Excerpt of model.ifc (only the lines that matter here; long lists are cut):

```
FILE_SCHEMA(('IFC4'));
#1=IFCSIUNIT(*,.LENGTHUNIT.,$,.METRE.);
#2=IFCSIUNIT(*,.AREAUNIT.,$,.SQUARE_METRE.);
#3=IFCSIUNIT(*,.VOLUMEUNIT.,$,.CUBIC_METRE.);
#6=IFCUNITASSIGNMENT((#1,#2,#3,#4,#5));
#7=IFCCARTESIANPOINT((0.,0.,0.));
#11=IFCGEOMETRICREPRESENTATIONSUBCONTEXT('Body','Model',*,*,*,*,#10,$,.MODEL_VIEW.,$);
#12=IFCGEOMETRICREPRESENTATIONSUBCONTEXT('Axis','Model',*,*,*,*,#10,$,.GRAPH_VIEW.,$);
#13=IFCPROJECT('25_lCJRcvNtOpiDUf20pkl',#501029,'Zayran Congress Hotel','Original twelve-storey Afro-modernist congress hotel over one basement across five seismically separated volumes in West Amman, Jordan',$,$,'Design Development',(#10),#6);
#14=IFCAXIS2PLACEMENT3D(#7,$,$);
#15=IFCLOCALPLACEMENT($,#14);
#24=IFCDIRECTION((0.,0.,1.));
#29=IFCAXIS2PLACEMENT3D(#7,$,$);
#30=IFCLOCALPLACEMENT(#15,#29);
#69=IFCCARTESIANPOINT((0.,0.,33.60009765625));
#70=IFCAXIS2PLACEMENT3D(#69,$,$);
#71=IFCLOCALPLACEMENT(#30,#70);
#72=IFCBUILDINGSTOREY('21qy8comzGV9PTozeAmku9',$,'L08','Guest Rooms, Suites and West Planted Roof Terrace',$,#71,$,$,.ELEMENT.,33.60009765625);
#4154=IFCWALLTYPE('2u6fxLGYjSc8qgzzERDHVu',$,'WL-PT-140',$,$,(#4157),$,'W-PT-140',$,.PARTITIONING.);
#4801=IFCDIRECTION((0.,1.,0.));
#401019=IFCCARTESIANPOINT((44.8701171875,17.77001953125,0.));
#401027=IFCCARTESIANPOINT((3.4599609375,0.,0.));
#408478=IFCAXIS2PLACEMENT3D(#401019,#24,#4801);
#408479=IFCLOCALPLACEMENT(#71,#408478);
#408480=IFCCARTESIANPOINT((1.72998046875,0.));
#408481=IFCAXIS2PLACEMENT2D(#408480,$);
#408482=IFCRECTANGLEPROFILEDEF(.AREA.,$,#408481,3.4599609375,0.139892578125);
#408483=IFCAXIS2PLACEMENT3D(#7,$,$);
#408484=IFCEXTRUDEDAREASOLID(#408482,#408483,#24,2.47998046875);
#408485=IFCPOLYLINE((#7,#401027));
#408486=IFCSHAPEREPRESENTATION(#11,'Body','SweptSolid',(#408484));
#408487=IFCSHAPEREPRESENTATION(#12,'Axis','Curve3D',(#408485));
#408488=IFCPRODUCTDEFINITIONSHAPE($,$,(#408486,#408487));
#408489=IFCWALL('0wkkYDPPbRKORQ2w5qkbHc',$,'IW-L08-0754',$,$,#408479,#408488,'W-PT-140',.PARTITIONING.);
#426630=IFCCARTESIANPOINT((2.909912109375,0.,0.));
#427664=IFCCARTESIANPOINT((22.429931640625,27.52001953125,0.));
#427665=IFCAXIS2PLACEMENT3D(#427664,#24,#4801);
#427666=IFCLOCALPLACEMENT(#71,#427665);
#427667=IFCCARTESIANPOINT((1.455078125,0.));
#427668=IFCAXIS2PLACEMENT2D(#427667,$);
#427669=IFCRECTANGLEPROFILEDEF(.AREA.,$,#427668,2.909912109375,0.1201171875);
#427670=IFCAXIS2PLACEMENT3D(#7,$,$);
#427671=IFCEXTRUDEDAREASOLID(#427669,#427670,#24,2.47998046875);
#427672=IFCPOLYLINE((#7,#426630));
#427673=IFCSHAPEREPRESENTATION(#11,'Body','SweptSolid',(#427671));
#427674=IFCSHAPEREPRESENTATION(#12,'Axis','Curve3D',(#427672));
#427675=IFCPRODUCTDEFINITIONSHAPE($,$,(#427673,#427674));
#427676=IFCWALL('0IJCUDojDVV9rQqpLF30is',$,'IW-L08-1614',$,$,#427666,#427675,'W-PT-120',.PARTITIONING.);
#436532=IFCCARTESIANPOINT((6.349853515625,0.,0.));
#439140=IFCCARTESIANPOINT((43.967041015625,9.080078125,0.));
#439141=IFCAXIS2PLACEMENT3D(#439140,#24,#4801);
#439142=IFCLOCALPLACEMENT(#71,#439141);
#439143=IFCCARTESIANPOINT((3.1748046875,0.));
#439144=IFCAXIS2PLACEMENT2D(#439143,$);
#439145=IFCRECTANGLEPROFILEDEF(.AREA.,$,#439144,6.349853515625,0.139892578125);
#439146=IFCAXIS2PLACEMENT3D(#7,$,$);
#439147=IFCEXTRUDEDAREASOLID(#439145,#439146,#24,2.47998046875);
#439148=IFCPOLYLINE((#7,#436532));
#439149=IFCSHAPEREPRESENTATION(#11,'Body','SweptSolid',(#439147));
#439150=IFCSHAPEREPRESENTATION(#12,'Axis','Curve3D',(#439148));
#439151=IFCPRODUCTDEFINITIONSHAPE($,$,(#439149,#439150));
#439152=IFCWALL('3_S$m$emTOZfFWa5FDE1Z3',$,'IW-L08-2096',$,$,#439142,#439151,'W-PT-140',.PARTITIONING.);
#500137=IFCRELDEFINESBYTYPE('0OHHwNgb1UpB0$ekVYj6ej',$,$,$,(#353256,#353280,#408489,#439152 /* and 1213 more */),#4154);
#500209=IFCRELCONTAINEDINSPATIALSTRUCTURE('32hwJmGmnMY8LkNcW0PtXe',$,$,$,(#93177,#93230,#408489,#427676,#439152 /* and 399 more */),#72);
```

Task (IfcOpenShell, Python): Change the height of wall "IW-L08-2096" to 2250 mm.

```python
import ifcopenshell
import ifcopenshell.geom
import ifcopenshell.util.representation
import ifcopenshell.util.shape
import ifcopenshell.util.unit

model = ifcopenshell.open("model.ifc")
unit_scale = ifcopenshell.util.unit.calculate_unit_scale(model)
settings = ifcopenshell.geom.settings()


def volume(element):
    """Net volume in cubic metres, openings subtracted."""
    shape = ifcopenshell.geom.create_shape(settings, element)
    return ifcopenshell.util.shape.get_volume(shape.geometry)


wall = model.by_id(439152)
before = volume(wall)

body = ifcopenshell.util.representation.get_representation(wall, "Model", "Body")
solid = body.Items[0]
old_height = solid.Depth
solid.Depth = 2.25 / unit_scale
after = volume(wall)

print(f"height {old_height:g} -> {solid.Depth:g}, volume {before:.3f} -> {after:.3f} m3")

model.write("model_v2.ifc")
```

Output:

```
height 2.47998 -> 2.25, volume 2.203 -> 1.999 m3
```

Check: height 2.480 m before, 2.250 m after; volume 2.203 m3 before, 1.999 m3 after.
